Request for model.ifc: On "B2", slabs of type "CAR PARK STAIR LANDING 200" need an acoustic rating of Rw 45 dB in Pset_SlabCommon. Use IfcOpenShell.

First a look at what the model holds.

```python
import ifcopenshell
import ifcopenshell.util.element

model = ifcopenshell.open("model.ifc")
print(model.schema)
storey = next(s for s in model.by_type("IfcBuildingStorey") if s.Name == "B2")
slabs = [e for e in ifcopenshell.util.element.get_decomposition(storey) if e.is_a("IfcSlab")]
seen = {}
for e in slabs:
    element_type = ifcopenshell.util.element.get_type(e)
    key = (element_type.Name if element_type != e and element_type else None, ifcopenshell.util.element.get_pset(e, "Pset_SlabCommon", "AcousticRating"))
    seen[key] = seen.get(key, 0) + 1
for (name, value), count in sorted(seen.items(), key=str):
    print(count, "x", name, "|", value)
```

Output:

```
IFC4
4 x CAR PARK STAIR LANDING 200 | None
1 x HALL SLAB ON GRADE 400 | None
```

```python
import ifcopenshell
import ifcopenshell.api.pset
import ifcopenshell.util.element

model = ifcopenshell.open("model.ifc")

storey = next(s for s in model.by_type("IfcBuildingStorey") if s.Name == "B2")
slabs = [e for e in ifcopenshell.util.element.get_decomposition(storey) if e.is_a("IfcSlab")]

count = 0
for e in slabs:
    element_type = ifcopenshell.util.element.get_type(e)
    if element_type in (None, e) or element_type.Name != "CAR PARK STAIR LANDING 200":
        continue
    found = ifcopenshell.util.element.get_pset(e, "Pset_SlabCommon", should_inherit=False)
    if found:
        pset = model.by_id(found["id"])
        if len(ifcopenshell.util.element.get_elements_by_pset(pset)) > 1:
            pset = ifcopenshell.api.pset.unshare_pset(model, products=[e], pset=pset)[0]
    else:
        pset = ifcopenshell.api.pset.add_pset(model, product=e, name="Pset_SlabCommon")
    ifcopenshell.api.pset.edit_pset(model, pset=pset, properties={"AcousticRating": "Rw 45 dB"})
    count += 1

print(count, "slabs updated")

model.write("model_edited.ifc")
```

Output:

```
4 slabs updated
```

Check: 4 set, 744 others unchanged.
